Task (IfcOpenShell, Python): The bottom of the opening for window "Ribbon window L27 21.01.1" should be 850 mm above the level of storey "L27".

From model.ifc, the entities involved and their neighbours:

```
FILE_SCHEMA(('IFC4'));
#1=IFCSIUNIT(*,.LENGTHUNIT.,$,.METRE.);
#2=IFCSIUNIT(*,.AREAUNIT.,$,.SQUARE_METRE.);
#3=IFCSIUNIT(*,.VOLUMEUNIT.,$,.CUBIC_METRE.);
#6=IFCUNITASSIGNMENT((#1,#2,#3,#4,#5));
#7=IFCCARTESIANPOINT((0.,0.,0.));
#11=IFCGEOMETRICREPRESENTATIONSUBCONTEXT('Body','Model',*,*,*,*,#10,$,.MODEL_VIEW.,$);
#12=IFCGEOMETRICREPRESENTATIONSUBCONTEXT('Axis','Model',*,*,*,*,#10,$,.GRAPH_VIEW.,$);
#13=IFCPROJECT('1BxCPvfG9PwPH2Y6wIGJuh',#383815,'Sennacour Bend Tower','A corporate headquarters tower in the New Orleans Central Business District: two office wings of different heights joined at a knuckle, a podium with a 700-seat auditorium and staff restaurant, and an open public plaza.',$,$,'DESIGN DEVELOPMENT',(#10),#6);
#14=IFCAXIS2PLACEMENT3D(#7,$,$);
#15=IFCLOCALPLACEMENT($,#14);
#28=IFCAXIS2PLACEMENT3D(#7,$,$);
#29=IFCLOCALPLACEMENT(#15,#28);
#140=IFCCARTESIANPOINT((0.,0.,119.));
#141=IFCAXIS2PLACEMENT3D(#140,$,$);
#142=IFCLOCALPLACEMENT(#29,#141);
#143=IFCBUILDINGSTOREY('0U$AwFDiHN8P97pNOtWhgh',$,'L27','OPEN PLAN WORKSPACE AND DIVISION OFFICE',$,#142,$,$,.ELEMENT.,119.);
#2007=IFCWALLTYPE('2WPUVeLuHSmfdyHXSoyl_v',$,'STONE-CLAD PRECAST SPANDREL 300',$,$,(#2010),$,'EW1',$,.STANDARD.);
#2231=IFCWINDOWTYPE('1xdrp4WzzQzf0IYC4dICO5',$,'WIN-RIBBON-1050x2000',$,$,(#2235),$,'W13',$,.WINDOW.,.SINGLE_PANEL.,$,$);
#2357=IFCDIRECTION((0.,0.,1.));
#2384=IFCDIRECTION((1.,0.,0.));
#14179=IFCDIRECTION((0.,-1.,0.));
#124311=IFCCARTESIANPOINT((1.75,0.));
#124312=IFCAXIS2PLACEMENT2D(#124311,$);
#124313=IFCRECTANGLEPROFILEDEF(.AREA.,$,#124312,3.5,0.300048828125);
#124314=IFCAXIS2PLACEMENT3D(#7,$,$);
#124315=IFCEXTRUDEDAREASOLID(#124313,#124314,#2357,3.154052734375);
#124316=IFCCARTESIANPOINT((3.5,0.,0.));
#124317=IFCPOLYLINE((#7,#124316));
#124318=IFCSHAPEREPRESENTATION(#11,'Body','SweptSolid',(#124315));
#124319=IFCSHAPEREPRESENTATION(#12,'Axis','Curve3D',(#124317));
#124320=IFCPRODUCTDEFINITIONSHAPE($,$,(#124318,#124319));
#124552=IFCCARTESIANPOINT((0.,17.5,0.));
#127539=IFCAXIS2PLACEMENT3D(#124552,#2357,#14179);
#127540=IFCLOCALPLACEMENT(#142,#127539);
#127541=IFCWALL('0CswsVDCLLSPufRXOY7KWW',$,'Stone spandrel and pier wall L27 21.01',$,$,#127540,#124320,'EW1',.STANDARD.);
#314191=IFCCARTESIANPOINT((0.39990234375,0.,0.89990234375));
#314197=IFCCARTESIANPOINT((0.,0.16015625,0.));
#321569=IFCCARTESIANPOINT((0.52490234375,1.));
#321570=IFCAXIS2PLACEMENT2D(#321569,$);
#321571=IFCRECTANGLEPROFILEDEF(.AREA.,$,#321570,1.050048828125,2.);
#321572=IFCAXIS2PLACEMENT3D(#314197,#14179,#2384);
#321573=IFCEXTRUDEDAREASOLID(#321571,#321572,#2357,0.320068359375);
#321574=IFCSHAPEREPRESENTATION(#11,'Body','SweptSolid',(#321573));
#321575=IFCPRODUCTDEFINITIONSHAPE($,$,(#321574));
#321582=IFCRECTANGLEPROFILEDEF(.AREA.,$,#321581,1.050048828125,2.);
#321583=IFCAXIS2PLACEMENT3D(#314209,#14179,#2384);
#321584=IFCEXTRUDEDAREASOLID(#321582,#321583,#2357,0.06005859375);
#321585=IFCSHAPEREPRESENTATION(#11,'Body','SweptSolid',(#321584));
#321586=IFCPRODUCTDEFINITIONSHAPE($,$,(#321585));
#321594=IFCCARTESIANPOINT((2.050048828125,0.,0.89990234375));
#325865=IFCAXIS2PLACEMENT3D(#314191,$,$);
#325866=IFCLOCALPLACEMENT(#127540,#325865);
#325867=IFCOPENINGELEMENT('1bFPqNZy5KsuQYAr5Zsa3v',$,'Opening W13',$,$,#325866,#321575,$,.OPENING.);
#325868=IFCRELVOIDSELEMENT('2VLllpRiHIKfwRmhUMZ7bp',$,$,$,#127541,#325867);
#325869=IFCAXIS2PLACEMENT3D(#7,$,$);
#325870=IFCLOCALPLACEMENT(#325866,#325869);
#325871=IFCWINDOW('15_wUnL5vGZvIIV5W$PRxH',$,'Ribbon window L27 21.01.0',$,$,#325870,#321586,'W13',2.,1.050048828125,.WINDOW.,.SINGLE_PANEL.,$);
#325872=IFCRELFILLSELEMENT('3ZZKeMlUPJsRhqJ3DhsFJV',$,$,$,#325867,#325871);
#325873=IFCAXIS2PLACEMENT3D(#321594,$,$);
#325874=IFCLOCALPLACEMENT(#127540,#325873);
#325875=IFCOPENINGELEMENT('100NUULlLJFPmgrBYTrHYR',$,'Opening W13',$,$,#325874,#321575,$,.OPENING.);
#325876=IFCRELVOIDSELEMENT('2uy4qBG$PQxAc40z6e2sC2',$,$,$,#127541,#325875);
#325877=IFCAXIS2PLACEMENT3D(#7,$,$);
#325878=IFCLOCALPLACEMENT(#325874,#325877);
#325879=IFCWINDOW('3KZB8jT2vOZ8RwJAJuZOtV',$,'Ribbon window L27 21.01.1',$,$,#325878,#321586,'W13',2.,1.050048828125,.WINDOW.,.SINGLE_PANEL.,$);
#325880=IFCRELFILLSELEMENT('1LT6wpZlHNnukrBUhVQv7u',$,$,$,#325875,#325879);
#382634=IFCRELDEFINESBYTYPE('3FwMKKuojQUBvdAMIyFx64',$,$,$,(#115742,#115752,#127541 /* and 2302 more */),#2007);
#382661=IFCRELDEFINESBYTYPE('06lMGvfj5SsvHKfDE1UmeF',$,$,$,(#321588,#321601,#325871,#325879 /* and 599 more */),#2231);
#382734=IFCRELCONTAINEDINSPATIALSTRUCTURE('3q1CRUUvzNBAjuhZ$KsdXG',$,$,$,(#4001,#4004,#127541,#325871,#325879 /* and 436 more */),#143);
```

```python
import numpy as np
import ifcopenshell
import ifcopenshell.api.geometry
import ifcopenshell.geom
import ifcopenshell.util.element
import ifcopenshell.util.placement
import ifcopenshell.util.shape
import ifcopenshell.util.unit

model = ifcopenshell.open("model.ifc")
unit_scale = ifcopenshell.util.unit.calculate_unit_scale(model)

window = model.by_guid("3KZB8jT2vOZ8RwJAJuZOtV")
opening = window.FillsVoids[0].RelatingOpeningElement
storey = ifcopenshell.util.element.get_container(window, ifc_class="IfcBuildingStorey")
level = ifcopenshell.util.placement.get_local_placement(storey.ObjectPlacement)[2, 3]

# The opening's origin need not be at the sill, so measure its lowest point.
shape = ifcopenshell.geom.create_shape(ifcopenshell.geom.settings(), opening)
bottom = ifcopenshell.util.shape.get_shape_bottom_elevation(shape, shape.geometry) / unit_scale
dz = level + 0.85 - bottom

shift = np.array([0.0, 0.0, dz])
# The window is placed relative to its opening, so it follows when the opening moves.
matrix = ifcopenshell.util.placement.get_local_placement(opening.ObjectPlacement)
matrix[:3, 3] += shift
ifcopenshell.api.geometry.edit_object_placement(
    model, product=opening, matrix=matrix, is_si=False, should_transform_children=True
)

print(f"moved by {dz * unit_scale:+.3f} m")

model.write("model_edited.ifc")
```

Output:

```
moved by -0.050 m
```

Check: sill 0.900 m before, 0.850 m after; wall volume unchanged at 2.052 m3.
